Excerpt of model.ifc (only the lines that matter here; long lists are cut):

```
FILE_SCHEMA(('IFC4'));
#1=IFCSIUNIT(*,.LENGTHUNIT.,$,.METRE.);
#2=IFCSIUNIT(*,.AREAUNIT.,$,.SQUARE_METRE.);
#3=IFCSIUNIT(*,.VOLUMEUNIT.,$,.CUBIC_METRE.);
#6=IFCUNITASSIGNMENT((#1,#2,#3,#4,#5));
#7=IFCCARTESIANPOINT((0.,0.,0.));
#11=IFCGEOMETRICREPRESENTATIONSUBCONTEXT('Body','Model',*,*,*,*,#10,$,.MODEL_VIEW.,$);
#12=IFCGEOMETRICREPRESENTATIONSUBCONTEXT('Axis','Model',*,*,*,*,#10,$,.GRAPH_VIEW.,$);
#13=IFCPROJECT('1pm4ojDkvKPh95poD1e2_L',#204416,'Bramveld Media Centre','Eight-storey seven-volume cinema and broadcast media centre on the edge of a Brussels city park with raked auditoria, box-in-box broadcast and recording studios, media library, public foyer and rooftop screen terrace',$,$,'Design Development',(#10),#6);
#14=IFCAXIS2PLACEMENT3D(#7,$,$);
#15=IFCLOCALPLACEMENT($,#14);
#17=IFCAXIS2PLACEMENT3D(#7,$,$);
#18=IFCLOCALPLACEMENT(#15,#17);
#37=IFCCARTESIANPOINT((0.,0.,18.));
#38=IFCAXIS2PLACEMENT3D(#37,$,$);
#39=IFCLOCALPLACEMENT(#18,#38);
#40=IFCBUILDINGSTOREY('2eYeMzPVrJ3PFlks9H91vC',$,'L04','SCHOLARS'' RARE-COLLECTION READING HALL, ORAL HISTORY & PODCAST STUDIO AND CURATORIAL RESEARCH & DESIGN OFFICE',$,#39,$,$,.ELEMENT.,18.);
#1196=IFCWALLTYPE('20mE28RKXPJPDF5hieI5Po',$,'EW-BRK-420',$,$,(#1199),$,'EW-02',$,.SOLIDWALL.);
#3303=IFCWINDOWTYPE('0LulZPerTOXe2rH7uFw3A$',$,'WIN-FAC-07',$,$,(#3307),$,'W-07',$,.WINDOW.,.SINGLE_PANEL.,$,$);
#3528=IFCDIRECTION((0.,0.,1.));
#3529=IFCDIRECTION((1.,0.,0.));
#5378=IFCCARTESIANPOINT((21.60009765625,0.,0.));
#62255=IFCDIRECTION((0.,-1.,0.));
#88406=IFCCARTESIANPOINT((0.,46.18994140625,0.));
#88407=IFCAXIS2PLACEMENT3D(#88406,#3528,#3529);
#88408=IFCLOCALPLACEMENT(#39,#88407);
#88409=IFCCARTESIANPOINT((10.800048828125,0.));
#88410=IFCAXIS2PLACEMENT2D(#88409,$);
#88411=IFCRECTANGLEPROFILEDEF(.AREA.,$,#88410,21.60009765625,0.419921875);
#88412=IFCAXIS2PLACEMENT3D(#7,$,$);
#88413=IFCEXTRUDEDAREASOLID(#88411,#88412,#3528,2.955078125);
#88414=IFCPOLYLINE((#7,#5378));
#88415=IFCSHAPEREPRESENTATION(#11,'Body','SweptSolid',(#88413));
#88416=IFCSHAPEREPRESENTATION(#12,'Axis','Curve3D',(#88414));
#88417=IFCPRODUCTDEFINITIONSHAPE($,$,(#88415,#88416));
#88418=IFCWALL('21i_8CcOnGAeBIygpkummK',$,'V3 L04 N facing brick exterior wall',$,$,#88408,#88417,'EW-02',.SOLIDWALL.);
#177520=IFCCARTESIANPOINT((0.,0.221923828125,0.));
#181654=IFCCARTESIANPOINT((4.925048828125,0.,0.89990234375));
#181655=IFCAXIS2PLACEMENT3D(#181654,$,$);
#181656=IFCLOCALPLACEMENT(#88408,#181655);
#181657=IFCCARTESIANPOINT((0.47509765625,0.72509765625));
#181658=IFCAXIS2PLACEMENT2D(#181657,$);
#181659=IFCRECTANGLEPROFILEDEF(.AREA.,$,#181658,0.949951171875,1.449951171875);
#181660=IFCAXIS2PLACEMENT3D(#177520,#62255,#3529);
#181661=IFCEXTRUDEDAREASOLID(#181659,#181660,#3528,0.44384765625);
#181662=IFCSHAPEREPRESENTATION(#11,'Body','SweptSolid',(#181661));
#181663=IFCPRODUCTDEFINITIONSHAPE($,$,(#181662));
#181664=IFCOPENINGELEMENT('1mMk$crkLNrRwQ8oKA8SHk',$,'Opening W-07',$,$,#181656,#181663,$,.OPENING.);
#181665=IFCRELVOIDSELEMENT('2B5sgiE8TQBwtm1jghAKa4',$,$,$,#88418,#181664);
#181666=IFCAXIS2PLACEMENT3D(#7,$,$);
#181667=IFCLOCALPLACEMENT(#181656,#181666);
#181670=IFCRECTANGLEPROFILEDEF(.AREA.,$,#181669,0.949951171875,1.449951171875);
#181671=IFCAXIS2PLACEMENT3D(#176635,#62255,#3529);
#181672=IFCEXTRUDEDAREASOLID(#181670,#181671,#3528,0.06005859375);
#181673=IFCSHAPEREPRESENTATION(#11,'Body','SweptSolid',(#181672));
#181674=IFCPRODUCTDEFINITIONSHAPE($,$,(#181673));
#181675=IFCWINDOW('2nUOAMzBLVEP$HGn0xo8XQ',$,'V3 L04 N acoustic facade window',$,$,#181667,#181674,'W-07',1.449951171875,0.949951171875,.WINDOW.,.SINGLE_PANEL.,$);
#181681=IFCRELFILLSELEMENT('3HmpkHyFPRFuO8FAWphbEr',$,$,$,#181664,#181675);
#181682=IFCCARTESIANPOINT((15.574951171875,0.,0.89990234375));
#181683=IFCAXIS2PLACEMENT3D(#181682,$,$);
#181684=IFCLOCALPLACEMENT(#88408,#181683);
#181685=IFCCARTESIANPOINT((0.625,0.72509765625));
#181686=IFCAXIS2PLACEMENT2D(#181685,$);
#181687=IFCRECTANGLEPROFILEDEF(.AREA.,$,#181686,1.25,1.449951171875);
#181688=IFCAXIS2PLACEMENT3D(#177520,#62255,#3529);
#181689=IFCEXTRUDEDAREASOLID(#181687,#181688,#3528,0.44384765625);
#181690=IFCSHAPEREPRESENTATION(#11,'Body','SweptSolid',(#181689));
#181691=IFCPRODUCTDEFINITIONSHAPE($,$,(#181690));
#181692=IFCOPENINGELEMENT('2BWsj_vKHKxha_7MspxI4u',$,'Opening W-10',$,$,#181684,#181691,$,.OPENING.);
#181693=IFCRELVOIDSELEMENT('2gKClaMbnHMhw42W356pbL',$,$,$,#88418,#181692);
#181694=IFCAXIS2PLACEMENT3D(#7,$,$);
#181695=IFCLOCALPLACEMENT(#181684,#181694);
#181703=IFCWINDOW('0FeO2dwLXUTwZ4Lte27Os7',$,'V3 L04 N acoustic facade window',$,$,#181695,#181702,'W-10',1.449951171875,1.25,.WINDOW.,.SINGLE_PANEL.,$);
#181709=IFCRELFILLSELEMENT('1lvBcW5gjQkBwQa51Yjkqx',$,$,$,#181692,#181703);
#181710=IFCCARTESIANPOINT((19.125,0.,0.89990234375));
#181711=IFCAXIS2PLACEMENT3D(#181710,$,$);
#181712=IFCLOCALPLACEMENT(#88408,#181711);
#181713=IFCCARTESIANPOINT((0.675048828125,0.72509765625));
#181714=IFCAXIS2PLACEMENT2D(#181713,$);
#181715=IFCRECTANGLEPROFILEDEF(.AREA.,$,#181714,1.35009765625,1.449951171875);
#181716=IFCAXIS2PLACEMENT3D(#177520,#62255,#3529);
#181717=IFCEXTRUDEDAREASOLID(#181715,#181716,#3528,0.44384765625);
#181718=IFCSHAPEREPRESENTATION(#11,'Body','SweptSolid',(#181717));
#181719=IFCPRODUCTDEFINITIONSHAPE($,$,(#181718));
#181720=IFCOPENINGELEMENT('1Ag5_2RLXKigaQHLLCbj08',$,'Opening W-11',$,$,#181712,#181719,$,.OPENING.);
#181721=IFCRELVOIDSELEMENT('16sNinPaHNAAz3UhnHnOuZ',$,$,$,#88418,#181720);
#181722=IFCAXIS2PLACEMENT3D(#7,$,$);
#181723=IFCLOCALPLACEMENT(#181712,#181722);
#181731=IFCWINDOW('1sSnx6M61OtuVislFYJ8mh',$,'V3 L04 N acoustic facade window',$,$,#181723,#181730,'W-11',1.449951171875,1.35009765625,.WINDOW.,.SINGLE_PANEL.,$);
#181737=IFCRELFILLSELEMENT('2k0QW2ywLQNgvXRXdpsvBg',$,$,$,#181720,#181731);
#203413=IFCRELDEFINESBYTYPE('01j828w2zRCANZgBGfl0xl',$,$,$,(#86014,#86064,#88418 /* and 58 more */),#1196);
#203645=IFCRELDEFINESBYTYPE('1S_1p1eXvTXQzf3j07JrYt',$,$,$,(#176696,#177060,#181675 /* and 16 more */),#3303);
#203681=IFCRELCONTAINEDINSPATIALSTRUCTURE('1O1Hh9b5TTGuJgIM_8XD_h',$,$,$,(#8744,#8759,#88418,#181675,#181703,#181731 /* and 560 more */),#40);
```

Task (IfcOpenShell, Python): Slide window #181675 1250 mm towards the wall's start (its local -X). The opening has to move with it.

```python
import ifcopenshell
import ifcopenshell.api.geometry
import ifcopenshell.util.placement
import ifcopenshell.util.unit

model = ifcopenshell.open("model.ifc")
unit_scale = ifcopenshell.util.unit.calculate_unit_scale(model)

window = model.by_guid("2nUOAMzBLVEP$HGn0xo8XQ")
opening = window.FillsVoids[0].RelatingOpeningElement
wall = opening.VoidsElements[0].RelatingBuildingElement

wall_matrix = ifcopenshell.util.placement.get_local_placement(wall.ObjectPlacement)
shift = wall_matrix[:3, 0] * -1.25 / unit_scale
before = ifcopenshell.util.placement.get_local_placement(window.ObjectPlacement)[:3, 3].copy()

# The window is placed relative to its opening, so it follows when the opening moves.
matrix = ifcopenshell.util.placement.get_local_placement(opening.ObjectPlacement)
matrix[:3, 3] += shift
ifcopenshell.api.geometry.edit_object_placement(
    model, product=opening, matrix=matrix, is_si=False, should_transform_children=True
)

after = ifcopenshell.util.placement.get_local_placement(window.ObjectPlacement)[:3, 3]
print("window moved by", (after - before).round(3) + 0.0)

model.write("model-out.ifc")
```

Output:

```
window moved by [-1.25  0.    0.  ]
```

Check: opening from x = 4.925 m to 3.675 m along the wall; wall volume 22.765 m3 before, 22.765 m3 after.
